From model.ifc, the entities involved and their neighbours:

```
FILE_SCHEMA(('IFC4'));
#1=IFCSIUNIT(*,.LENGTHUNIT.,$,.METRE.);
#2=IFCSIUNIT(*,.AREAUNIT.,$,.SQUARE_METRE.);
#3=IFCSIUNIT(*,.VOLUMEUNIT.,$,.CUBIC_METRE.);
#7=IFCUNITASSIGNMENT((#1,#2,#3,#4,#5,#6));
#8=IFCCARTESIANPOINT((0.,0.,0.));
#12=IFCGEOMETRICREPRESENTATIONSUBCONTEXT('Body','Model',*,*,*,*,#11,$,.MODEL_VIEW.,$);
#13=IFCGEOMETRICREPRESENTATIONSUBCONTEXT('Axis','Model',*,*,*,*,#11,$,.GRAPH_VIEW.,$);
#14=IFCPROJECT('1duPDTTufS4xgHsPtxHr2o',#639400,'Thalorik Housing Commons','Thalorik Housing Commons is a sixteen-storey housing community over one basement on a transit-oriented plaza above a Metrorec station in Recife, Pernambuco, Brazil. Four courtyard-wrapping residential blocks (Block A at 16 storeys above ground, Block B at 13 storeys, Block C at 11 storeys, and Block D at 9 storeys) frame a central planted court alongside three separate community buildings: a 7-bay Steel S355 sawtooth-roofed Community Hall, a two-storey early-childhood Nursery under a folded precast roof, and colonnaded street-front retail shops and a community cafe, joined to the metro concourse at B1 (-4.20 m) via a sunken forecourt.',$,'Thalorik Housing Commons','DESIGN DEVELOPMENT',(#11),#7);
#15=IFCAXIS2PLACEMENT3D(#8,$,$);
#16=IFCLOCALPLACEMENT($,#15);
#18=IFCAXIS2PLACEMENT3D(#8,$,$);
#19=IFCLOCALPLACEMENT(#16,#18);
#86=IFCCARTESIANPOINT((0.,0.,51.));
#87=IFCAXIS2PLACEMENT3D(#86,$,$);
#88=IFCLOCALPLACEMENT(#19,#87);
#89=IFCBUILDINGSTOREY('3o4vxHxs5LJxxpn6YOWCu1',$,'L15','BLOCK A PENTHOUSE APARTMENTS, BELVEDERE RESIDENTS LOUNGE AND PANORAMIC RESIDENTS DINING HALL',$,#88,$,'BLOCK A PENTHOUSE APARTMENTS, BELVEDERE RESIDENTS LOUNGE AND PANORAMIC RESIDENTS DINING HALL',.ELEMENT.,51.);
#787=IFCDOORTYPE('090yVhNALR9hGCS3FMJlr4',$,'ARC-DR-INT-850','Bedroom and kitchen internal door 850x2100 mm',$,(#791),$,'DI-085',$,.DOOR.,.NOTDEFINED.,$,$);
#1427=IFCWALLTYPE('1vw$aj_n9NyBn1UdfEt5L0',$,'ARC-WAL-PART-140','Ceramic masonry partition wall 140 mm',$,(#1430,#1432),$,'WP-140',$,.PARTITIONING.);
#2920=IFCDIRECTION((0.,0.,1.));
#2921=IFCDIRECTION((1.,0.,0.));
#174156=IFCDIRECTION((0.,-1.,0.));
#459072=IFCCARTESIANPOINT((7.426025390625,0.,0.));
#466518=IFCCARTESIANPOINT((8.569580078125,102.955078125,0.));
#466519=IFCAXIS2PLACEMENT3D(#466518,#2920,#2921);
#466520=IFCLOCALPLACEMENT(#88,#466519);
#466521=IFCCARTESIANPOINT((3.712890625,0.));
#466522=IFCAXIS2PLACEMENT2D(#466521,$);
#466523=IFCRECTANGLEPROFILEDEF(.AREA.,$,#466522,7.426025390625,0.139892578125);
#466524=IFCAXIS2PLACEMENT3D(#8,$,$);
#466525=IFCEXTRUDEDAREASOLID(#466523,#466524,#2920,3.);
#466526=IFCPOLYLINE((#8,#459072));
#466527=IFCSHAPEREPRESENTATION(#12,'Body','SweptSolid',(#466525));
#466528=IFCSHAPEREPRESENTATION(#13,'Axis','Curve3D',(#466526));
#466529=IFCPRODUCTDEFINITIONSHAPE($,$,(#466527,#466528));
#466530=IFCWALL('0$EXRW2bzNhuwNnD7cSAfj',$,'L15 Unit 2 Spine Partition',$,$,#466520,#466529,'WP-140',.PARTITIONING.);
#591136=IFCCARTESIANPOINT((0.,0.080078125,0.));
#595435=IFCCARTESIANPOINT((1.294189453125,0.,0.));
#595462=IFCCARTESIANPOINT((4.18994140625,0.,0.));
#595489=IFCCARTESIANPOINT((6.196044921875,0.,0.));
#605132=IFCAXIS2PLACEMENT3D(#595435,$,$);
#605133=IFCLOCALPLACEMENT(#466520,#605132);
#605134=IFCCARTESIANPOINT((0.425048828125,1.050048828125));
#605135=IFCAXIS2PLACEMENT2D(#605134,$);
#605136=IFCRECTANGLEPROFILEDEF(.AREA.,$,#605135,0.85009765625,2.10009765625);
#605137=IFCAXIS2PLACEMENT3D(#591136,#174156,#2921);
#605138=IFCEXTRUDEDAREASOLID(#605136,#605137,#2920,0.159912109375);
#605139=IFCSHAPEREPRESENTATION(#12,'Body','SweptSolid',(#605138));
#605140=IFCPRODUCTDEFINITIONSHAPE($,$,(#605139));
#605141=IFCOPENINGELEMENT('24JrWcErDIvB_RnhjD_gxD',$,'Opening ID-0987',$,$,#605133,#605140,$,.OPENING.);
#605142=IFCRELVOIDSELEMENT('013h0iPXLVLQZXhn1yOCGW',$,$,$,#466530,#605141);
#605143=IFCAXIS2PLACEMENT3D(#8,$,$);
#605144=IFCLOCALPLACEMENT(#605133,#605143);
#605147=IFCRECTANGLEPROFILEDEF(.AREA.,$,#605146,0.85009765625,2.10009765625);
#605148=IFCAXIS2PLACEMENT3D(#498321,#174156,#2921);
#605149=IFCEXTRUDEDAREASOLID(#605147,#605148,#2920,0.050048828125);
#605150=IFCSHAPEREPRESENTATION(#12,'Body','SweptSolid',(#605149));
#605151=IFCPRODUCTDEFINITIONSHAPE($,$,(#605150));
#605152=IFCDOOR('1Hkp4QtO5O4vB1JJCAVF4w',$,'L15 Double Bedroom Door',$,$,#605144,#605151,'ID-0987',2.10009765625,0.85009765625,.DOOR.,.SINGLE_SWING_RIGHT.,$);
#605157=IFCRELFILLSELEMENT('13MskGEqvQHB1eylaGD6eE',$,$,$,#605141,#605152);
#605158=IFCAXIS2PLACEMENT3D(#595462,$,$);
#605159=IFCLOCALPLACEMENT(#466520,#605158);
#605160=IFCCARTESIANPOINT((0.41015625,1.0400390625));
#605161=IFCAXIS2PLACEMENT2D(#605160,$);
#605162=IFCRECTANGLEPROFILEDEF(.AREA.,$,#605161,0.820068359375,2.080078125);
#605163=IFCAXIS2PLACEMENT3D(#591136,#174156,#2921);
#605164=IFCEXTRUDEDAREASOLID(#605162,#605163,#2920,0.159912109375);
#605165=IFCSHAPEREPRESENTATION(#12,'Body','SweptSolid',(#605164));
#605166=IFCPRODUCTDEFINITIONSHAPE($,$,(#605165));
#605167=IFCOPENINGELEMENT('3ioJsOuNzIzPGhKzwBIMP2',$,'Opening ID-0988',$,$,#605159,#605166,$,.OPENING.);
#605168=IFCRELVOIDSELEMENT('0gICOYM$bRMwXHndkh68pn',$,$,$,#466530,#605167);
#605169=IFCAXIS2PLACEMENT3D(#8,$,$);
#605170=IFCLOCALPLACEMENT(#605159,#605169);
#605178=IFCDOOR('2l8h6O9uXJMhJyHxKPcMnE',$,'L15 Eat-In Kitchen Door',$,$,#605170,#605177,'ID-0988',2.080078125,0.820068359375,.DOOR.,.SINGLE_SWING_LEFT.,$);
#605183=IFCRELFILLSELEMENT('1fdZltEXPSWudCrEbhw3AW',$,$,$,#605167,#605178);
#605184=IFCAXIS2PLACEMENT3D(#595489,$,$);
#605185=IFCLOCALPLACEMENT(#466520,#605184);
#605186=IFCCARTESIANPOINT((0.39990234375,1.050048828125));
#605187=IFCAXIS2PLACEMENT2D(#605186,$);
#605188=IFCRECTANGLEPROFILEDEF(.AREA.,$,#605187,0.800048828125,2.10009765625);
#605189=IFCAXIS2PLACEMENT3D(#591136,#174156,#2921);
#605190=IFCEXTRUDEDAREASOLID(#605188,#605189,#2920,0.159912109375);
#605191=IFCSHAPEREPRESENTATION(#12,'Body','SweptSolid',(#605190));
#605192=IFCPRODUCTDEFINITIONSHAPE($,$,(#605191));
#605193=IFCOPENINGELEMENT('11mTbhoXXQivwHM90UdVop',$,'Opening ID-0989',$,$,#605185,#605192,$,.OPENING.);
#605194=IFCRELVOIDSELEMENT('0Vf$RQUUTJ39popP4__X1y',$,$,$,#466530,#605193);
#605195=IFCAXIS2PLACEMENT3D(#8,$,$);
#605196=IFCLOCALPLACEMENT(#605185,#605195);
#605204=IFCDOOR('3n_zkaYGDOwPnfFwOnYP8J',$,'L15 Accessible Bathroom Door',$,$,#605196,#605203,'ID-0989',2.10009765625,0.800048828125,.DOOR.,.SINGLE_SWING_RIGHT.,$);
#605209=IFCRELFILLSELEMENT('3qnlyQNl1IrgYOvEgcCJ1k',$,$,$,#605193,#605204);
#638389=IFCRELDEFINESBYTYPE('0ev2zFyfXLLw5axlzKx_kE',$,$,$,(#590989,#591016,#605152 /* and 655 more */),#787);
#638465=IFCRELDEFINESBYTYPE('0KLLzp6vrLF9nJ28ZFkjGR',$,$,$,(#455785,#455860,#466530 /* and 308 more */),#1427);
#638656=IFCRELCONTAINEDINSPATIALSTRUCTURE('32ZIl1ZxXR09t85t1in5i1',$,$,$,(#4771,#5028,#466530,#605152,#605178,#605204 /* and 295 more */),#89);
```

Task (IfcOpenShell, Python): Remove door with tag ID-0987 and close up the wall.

```python
import ifcopenshell
import ifcopenshell.api.feature
import ifcopenshell.api.root
import ifcopenshell.geom
import ifcopenshell.util.shape

model = ifcopenshell.open("model.ifc")
settings = ifcopenshell.geom.settings()


def volume(element):
    """Net volume in cubic metres, openings subtracted."""
    shape = ifcopenshell.geom.create_shape(settings, element)
    return ifcopenshell.util.shape.get_volume(shape.geometry)


door = model.by_guid("1Hkp4QtO5O4vB1JJCAVF4w")
opening = door.FillsVoids[0].RelatingOpeningElement
wall = opening.VoidsElements[0].RelatingBuildingElement
before = volume(wall)

ifcopenshell.api.root.remove_product(model, product=door)
ifcopenshell.api.feature.remove_feature(model, feature=opening)

after = volume(wall)

print(f"wall volume {before:.3f} -> {after:.3f} m3")

model.write("model_v2.ifc")
```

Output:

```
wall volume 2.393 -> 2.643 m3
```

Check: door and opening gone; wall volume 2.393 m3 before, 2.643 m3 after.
